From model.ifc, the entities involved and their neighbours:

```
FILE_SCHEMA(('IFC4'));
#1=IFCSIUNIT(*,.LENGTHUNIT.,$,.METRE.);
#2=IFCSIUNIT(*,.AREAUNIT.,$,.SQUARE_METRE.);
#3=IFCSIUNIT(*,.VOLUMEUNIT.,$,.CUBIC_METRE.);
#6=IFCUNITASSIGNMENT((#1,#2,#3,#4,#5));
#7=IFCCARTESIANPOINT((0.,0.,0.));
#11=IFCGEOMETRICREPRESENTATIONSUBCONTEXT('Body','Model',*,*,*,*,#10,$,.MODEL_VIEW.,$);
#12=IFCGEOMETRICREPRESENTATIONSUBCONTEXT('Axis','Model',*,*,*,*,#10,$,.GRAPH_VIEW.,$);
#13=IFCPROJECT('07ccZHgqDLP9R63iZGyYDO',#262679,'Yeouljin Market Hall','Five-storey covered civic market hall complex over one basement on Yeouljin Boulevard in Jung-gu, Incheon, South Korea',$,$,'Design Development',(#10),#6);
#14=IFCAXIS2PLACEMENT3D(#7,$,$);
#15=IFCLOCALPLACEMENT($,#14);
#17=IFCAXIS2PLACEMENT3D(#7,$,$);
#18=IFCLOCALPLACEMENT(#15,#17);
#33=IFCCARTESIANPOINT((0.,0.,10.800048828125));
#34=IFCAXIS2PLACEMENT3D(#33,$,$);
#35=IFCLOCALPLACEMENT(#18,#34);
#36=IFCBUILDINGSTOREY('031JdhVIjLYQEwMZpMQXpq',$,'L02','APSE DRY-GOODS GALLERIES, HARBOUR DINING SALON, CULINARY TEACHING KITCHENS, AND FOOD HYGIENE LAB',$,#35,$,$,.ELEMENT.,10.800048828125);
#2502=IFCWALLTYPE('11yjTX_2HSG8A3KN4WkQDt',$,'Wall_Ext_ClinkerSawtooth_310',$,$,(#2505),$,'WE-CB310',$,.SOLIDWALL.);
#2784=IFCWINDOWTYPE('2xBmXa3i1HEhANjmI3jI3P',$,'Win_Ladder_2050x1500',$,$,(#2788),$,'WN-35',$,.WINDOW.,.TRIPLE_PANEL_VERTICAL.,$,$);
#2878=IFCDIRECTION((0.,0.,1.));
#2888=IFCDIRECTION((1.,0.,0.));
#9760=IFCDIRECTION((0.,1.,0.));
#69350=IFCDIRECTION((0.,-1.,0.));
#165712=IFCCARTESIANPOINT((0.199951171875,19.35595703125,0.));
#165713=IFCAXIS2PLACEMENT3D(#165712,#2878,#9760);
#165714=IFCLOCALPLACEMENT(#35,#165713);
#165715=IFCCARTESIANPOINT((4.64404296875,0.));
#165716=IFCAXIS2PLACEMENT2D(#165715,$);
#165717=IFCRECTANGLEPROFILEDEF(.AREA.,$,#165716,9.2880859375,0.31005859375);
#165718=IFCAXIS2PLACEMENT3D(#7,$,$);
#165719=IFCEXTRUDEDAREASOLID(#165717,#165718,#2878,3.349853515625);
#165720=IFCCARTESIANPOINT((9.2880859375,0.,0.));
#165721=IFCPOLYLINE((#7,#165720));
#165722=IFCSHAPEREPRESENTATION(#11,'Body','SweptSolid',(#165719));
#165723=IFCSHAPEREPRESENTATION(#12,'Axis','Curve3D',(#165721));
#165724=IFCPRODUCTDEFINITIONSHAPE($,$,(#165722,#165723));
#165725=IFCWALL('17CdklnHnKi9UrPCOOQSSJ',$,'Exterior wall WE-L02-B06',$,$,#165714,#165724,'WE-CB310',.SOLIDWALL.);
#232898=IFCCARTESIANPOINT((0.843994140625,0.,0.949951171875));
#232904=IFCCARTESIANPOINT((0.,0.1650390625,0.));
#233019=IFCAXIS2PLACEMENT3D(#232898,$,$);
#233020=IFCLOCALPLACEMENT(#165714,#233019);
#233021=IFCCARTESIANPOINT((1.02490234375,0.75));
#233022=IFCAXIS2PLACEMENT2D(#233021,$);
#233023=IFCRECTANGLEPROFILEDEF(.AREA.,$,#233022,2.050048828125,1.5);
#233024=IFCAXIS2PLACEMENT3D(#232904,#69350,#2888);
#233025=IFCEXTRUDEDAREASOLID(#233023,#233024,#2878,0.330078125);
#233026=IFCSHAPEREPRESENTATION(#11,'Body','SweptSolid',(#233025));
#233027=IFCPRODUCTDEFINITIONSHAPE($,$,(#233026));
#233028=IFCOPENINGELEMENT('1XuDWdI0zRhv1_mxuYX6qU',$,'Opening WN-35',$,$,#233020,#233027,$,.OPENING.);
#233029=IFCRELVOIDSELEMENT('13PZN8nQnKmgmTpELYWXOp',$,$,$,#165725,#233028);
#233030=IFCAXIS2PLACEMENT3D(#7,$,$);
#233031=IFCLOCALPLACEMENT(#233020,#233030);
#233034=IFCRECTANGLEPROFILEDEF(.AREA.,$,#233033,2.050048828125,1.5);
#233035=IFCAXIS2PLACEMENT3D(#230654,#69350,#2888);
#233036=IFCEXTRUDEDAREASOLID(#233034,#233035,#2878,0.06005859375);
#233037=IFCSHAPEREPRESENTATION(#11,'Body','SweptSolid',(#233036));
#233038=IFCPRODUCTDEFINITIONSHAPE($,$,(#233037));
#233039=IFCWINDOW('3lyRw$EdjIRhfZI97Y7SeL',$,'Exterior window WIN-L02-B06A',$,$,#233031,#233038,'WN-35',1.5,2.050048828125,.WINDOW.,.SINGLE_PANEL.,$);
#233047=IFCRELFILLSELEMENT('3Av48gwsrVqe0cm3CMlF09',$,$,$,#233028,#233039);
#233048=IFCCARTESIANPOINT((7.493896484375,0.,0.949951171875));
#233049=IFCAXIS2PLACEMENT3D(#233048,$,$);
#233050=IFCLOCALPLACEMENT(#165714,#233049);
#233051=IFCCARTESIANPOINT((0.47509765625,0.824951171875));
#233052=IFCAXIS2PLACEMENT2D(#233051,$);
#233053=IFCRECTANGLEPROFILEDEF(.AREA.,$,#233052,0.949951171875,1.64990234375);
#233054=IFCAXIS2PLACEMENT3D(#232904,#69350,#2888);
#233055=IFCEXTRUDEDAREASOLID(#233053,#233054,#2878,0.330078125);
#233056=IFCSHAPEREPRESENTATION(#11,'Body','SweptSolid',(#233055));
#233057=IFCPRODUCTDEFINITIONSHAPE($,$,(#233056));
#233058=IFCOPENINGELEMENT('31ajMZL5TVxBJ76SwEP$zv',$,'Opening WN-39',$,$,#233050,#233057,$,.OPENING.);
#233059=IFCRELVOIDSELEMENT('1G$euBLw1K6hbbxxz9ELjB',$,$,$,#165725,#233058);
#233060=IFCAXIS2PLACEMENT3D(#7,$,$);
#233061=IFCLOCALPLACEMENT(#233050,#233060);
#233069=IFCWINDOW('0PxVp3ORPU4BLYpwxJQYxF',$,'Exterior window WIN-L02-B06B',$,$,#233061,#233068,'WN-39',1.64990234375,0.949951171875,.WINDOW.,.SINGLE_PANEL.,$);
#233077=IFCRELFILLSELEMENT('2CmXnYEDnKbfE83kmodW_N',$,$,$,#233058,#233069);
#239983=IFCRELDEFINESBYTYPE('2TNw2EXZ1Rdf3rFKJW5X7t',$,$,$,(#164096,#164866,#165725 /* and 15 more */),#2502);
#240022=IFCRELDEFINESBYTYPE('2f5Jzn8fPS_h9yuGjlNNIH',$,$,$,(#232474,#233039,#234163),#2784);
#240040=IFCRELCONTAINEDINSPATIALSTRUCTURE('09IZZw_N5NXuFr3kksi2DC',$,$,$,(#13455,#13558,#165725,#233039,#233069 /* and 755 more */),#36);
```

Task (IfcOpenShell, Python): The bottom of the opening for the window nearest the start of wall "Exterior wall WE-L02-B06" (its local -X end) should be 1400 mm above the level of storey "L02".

```python
import numpy as np
import ifcopenshell
import ifcopenshell.api.geometry
import ifcopenshell.geom
import ifcopenshell.util.element
import ifcopenshell.util.placement
import ifcopenshell.util.shape
import ifcopenshell.util.unit

model = ifcopenshell.open("model.ifc")
unit_scale = ifcopenshell.util.unit.calculate_unit_scale(model)

window = model.by_guid("3lyRw$EdjIRhfZI97Y7SeL")
opening = window.FillsVoids[0].RelatingOpeningElement
storey = ifcopenshell.util.element.get_container(window, ifc_class="IfcBuildingStorey")
level = ifcopenshell.util.placement.get_local_placement(storey.ObjectPlacement)[2, 3]

# The opening's origin need not be at the sill, so measure its lowest point.
shape = ifcopenshell.geom.create_shape(ifcopenshell.geom.settings(), opening)
bottom = ifcopenshell.util.shape.get_shape_bottom_elevation(shape, shape.geometry) / unit_scale
dz = level + 1.4 - bottom

shift = np.array([0.0, 0.0, dz])
# The window is placed relative to its opening, so it follows when the opening moves.
matrix = ifcopenshell.util.placement.get_local_placement(opening.ObjectPlacement)
matrix[:3, 3] += shift
ifcopenshell.api.geometry.edit_object_placement(
    model, product=opening, matrix=matrix, is_si=False, should_transform_children=True
)

print(f"moved by {dz * unit_scale:+.3f} m")

model.write("model-out.ifc")
```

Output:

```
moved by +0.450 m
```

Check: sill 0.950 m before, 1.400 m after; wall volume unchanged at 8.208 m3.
